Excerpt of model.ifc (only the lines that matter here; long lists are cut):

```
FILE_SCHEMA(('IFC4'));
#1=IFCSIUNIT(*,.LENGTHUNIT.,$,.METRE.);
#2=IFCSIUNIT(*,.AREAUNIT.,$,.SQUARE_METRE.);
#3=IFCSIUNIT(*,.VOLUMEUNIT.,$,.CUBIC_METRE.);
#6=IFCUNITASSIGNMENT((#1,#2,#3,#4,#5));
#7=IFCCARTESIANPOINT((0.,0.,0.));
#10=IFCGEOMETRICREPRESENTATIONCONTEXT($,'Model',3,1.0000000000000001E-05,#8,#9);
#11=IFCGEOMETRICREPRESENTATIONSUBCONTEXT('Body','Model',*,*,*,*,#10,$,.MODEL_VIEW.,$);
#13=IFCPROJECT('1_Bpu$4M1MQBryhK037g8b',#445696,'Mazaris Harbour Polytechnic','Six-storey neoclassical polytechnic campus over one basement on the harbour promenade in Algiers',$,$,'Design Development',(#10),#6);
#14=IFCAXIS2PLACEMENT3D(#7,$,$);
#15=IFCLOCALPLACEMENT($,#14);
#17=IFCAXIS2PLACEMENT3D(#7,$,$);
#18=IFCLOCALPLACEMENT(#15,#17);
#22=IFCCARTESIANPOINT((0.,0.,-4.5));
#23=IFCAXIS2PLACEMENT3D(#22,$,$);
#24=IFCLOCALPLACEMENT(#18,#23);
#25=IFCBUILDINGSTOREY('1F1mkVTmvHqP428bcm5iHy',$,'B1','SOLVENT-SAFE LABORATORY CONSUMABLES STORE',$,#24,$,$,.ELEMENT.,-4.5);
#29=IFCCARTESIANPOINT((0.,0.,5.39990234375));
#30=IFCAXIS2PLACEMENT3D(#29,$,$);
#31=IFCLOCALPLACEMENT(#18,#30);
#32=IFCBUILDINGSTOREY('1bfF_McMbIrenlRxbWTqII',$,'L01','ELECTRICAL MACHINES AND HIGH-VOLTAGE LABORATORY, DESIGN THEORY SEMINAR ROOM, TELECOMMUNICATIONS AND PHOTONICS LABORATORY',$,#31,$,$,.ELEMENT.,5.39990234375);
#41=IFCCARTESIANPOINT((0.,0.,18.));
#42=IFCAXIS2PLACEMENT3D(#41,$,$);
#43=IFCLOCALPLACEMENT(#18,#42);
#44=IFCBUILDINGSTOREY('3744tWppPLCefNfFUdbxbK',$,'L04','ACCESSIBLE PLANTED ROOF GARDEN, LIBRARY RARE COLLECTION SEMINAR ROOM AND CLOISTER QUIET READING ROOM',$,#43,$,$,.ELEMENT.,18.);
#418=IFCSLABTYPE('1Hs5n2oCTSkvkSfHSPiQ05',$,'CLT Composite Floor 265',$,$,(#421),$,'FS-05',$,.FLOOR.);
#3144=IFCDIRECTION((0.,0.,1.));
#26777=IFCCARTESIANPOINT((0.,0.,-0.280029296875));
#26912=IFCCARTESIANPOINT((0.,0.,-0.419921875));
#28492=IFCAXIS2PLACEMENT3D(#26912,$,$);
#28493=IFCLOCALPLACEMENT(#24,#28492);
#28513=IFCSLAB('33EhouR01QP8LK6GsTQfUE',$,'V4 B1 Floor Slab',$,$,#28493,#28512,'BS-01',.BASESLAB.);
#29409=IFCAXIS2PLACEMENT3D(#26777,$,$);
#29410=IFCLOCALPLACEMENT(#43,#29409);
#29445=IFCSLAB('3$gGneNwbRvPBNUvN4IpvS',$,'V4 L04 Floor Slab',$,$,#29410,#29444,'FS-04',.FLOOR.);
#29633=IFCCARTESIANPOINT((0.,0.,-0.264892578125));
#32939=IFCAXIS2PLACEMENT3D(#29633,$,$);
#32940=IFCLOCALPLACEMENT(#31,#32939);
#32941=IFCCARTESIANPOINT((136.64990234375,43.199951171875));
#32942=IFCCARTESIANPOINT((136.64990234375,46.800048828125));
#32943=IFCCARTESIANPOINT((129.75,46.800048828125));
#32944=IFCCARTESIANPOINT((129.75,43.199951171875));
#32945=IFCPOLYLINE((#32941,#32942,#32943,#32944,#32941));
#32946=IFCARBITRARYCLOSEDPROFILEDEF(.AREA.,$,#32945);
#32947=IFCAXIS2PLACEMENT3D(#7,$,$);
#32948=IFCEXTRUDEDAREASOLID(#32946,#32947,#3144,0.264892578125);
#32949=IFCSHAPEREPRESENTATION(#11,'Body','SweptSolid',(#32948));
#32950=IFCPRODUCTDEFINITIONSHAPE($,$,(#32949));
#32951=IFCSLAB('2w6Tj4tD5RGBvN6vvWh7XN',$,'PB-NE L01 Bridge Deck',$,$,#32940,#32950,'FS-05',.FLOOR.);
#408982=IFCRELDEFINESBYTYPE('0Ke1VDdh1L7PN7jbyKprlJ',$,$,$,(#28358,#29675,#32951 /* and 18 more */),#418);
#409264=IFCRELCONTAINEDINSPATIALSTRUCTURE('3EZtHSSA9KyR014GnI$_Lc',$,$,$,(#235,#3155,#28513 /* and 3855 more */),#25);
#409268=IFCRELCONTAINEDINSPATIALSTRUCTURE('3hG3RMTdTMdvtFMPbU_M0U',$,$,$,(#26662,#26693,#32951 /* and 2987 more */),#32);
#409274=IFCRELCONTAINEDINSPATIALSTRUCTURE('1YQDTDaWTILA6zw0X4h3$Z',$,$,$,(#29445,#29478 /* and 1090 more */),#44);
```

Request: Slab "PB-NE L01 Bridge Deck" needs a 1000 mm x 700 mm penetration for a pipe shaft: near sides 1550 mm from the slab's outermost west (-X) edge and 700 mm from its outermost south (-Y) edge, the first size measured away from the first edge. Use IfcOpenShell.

```python
import numpy as np
import ifcopenshell
import ifcopenshell.api.feature
import ifcopenshell.api.geometry
import ifcopenshell.api.root
import ifcopenshell.geom
import ifcopenshell.util.placement
import ifcopenshell.util.representation
import ifcopenshell.util.shape
import ifcopenshell.util.unit

model = ifcopenshell.open("model.ifc")
unit_scale = ifcopenshell.util.unit.calculate_unit_scale(model)
settings = ifcopenshell.geom.settings()


def volume(element):
    """Net volume in cubic metres, openings subtracted."""
    shape = ifcopenshell.geom.create_shape(settings, element)
    return ifcopenshell.util.shape.get_volume(shape.geometry)


slab = model.by_guid("2w6Tj4tD5RGBvN6vvWh7XN")
before = volume(slab)

# Extent in the slab's own axes, in metres. The edges named are its -X and -Y sides.
slab_shape = ifcopenshell.geom.create_shape(settings, slab)
vertices = ifcopenshell.util.shape.get_vertices(slab_shape.geometry)
x_min, y_min, bottom = vertices.min(axis=0)
top = vertices[:, 2].max()

opening = ifcopenshell.api.root.create_entity(model, ifc_class="IfcOpeningElement", name="Pipe shaft opening", predefined_type="OPENING")
context = ifcopenshell.util.representation.get_context(model, "Model", "Body", "MODEL_VIEW")
width, depth = 1, 0.7
outline = [(0.0, 0.0), (width, 0.0), (width, depth), (0.0, depth), (0.0, 0.0)]
# Overshoot both faces by 50 mm so the cut is clean.
shape = ifcopenshell.api.geometry.add_slab_representation(
    model, context=context, depth=top - bottom + 0.1, polyline=outline
)
ifcopenshell.api.geometry.assign_representation(model, product=opening, representation=shape)

matrix = ifcopenshell.util.placement.get_local_placement(slab.ObjectPlacement)
matrix[:, 3] = matrix @ np.append(np.array([x_min + 1.55, y_min + 0.7, bottom - 0.05]) / unit_scale, 1.0)
ifcopenshell.api.geometry.edit_object_placement(model, product=opening, matrix=matrix, is_si=False)
ifcopenshell.api.feature.add_feature(model, feature=opening, element=slab)

after = volume(slab)

print(f"slab volume {before:.3f} -> {after:.3f} m3")

model.write("model_v2.ifc")
```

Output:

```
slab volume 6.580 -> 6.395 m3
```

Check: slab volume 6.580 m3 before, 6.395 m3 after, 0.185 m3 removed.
